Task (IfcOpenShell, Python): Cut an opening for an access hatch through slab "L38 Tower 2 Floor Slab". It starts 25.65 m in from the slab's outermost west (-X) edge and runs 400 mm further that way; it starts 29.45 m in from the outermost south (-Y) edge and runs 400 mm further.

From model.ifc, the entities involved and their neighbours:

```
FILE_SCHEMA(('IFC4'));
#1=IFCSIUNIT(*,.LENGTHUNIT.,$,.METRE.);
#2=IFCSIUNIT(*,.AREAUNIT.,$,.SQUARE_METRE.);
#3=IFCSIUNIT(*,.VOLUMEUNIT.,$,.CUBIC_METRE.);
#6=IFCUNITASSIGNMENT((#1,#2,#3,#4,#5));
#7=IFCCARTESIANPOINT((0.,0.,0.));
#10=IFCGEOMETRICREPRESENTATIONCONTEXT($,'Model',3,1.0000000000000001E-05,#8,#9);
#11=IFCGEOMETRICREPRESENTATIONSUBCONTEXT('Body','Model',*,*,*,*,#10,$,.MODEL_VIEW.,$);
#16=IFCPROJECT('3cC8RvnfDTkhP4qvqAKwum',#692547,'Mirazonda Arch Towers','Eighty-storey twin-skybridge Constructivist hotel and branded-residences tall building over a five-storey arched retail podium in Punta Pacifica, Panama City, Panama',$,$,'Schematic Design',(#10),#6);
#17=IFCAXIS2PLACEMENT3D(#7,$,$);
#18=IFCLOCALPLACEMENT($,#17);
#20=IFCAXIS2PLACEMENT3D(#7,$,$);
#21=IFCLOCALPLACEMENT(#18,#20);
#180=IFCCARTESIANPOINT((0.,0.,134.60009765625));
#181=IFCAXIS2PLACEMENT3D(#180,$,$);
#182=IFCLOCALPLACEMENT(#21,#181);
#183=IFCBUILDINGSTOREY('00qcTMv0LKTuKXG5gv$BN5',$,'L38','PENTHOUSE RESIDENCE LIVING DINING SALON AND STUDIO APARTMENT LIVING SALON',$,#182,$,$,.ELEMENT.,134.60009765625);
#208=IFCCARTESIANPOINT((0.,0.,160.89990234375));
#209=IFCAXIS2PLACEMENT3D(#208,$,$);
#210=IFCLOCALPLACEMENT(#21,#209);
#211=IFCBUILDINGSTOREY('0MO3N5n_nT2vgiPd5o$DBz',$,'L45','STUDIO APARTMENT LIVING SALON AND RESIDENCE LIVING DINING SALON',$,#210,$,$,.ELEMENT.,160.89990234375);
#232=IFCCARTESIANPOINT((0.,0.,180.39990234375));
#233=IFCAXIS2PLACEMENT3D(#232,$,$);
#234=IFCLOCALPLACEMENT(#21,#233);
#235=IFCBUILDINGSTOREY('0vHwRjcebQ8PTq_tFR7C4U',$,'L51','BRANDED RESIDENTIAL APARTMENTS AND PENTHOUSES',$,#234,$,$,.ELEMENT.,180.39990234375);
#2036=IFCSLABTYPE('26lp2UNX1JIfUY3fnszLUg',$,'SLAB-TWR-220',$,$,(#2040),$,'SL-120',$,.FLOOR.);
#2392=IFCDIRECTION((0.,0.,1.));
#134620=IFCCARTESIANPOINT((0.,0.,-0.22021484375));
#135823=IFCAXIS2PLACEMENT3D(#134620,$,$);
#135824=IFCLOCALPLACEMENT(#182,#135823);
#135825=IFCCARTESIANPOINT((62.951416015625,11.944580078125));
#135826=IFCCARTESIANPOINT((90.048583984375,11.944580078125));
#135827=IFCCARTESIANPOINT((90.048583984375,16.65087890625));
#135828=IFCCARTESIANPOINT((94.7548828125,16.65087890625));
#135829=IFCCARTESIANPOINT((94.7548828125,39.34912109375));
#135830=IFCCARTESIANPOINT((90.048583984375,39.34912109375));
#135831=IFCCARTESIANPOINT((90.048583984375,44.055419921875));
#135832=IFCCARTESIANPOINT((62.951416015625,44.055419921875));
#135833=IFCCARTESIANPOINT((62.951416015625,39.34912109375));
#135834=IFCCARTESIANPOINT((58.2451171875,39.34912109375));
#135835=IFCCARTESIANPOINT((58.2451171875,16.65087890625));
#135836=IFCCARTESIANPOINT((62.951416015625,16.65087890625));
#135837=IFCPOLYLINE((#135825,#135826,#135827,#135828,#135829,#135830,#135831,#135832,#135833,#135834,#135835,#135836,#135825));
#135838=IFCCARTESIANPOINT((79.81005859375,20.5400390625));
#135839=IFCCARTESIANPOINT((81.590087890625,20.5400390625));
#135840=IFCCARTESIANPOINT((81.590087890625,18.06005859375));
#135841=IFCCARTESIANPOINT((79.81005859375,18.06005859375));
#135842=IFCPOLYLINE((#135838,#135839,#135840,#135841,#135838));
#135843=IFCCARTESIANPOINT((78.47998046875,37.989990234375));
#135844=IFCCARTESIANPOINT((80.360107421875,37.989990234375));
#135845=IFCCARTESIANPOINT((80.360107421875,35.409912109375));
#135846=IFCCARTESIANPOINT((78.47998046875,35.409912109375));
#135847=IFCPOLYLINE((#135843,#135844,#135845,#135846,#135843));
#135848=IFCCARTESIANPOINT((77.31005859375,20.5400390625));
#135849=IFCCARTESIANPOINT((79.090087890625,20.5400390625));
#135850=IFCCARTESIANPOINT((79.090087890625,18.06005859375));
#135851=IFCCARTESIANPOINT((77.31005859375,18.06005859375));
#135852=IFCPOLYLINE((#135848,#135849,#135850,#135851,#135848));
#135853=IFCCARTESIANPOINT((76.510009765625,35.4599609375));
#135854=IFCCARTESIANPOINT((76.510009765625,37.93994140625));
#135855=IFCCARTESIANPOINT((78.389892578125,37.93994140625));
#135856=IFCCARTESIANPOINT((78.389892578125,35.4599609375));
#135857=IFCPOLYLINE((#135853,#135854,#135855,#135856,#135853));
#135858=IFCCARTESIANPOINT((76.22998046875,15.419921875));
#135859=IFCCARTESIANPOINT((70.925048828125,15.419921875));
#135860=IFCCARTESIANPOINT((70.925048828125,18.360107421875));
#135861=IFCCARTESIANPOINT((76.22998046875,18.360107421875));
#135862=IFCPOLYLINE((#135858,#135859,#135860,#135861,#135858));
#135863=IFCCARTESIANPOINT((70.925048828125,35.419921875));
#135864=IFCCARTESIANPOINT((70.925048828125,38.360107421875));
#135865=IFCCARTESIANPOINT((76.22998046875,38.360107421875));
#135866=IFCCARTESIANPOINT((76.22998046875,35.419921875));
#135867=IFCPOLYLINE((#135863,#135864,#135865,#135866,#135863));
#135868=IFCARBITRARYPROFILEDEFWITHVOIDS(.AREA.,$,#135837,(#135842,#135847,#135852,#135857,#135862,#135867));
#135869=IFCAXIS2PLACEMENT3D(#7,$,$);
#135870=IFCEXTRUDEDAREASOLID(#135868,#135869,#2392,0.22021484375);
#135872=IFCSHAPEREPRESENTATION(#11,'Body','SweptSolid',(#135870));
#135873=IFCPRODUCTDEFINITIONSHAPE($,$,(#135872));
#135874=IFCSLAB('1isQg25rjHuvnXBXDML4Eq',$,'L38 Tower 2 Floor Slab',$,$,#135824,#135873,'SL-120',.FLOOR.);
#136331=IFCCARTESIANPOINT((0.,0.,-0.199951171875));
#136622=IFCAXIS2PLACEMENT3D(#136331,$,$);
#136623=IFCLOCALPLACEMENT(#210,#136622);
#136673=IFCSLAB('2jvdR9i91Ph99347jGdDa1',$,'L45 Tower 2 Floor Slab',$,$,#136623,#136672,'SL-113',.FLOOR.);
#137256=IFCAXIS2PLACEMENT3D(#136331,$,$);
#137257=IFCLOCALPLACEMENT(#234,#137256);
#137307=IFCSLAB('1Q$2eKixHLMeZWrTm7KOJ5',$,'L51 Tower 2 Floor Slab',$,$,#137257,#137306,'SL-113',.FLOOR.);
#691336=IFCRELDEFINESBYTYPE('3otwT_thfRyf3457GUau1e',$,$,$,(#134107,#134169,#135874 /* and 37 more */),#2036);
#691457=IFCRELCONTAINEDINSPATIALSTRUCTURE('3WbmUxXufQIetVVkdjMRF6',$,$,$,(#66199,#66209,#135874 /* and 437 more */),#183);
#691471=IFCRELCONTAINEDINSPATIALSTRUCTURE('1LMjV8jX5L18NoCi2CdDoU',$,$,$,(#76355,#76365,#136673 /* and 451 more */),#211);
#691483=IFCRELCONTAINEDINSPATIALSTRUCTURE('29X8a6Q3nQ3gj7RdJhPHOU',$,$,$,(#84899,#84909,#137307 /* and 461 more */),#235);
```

```python
import numpy as np
import ifcopenshell
import ifcopenshell.api.feature
import ifcopenshell.api.geometry
import ifcopenshell.api.root
import ifcopenshell.geom
import ifcopenshell.util.placement
import ifcopenshell.util.representation
import ifcopenshell.util.shape
import ifcopenshell.util.unit

model = ifcopenshell.open("model.ifc")
unit_scale = ifcopenshell.util.unit.calculate_unit_scale(model)
settings = ifcopenshell.geom.settings()


def volume(element):
    """Net volume in cubic metres, openings subtracted."""
    shape = ifcopenshell.geom.create_shape(settings, element)
    return ifcopenshell.util.shape.get_volume(shape.geometry)


slab = model.by_guid("1isQg25rjHuvnXBXDML4Eq")
before = volume(slab)

# Extent in the slab's own axes, in metres. The edges named are its -X and -Y sides.
slab_shape = ifcopenshell.geom.create_shape(settings, slab)
vertices = ifcopenshell.util.shape.get_vertices(slab_shape.geometry)
x_min, y_min, bottom = vertices.min(axis=0)
top = vertices[:, 2].max()

opening = ifcopenshell.api.root.create_entity(model, ifc_class="IfcOpeningElement", name="Access hatch opening", predefined_type="OPENING")
context = ifcopenshell.util.representation.get_context(model, "Model", "Body", "MODEL_VIEW")
width, depth = 0.4, 0.4
outline = [(0.0, 0.0), (width, 0.0), (width, depth), (0.0, depth), (0.0, 0.0)]
# Overshoot both faces by 50 mm so the cut is clean.
shape = ifcopenshell.api.geometry.add_slab_representation(
    model, context=context, depth=top - bottom + 0.1, polyline=outline
)
ifcopenshell.api.geometry.assign_representation(model, product=opening, representation=shape)

matrix = ifcopenshell.util.placement.get_local_placement(slab.ObjectPlacement)
matrix[:, 3] = matrix @ np.append(np.array([x_min + 25.65, y_min + 29.45, bottom - 0.05]) / unit_scale, 1.0)
ifcopenshell.api.geometry.edit_object_placement(model, product=opening, matrix=matrix, is_si=False)
ifcopenshell.api.feature.add_feature(model, feature=opening, element=slab)

after = volume(slab)

print(f"slab volume {before:.3f} -> {after:.3f} m3")

model.write("model_edited.ifc")
```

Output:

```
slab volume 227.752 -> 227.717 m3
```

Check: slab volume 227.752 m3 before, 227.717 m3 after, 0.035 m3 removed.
